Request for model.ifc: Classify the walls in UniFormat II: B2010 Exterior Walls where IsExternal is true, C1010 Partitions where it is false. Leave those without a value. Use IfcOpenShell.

First a look at what the model holds.

```python
import ifcopenshell
import ifcopenshell.util.element

model = ifcopenshell.open("model.ifc")
print(model.schema)
print("classifications:", [c.Name for c in model.by_type("IfcClassification")])
values = [ifcopenshell.util.element.get_pset(e, "Pset_WallCommon", "IsExternal") for e in model.by_type("IfcWall")]
for value in (True, False, None):
    print("IsExternal", value, values.count(value))
```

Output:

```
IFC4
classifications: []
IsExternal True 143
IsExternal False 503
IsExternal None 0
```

```python
import ifcopenshell
import ifcopenshell.api.classification
import ifcopenshell.util.element

model = ifcopenshell.open("model.ifc")

system = ifcopenshell.api.classification.add_classification(model, classification="UniFormat II")

walls = model.by_type("IfcWall")
external = {e: ifcopenshell.util.element.get_pset(e, "Pset_WallCommon", "IsExternal") for e in walls}
for flag, code, name in ((True, "B2010", "Exterior Walls"), (False, "C1010", "Partitions")):
    products = [e for e in walls if external[e] is flag]
    ifcopenshell.api.classification.add_reference(
        model, products=products, classification=system, identification=code, name=name
    )
    print(code, len(products))

model.write("model_rev.ifc")
```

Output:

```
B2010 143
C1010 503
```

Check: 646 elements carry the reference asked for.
